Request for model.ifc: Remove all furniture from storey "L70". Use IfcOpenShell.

First a look at what the model holds.

```python
import ifcopenshell
import ifcopenshell.util.element

model = ifcopenshell.open("model.ifc")
print(model.schema)
storey = next(s for s in model.by_type("IfcBuildingStorey") if s.Name == "L70")
furniture = [e for e in ifcopenshell.util.element.get_decomposition(storey) if e.is_a("IfcFurnishingElement")]
seen = {}
for e in furniture:
    element_type = ifcopenshell.util.element.get_type(e)
    name = element_type.Name if element_type not in (None, e) else None
    seen[name] = seen.get(name, 0) + 1
for name, count in sorted(seen.items(), key=str):
    print(count, "x", name)
```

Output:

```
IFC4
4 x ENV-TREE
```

```python
import ifcopenshell
import ifcopenshell.api.root
import ifcopenshell.util.element

model = ifcopenshell.open("model.ifc")

storey = next(s for s in model.by_type("IfcBuildingStorey") if s.Name == "L70")
furniture = [e for e in ifcopenshell.util.element.get_decomposition(storey) if e.is_a("IfcFurnishingElement")]

for e in furniture:
    ifcopenshell.api.root.remove_product(model, product=e)
print(len(furniture), "removed")

model.write("model_v2.ifc")
```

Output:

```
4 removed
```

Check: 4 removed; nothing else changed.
